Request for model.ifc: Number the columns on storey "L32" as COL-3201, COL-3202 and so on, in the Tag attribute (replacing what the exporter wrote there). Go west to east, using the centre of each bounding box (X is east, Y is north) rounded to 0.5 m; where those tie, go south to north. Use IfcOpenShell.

First a look at what the model holds.

```python
import ifcopenshell
import ifcopenshell.util.element
import ifcopenshell.util.placement

model = ifcopenshell.open("model.ifc")
print(model.schema)
storey = next(s for s in model.by_type("IfcBuildingStorey") if s.Name == "L32")
columns = [e for e in ifcopenshell.util.element.get_decomposition(storey) if e.is_a("IfcColumn")]
for e in sorted(columns, key=lambda e: e.id()):
    origin = ifcopenshell.util.placement.get_local_placement(e.ObjectPlacement)[:3, 3]
    print(e.id(), e.Tag, e.Name, origin.round(2) + 0.0, sep=" | ")
```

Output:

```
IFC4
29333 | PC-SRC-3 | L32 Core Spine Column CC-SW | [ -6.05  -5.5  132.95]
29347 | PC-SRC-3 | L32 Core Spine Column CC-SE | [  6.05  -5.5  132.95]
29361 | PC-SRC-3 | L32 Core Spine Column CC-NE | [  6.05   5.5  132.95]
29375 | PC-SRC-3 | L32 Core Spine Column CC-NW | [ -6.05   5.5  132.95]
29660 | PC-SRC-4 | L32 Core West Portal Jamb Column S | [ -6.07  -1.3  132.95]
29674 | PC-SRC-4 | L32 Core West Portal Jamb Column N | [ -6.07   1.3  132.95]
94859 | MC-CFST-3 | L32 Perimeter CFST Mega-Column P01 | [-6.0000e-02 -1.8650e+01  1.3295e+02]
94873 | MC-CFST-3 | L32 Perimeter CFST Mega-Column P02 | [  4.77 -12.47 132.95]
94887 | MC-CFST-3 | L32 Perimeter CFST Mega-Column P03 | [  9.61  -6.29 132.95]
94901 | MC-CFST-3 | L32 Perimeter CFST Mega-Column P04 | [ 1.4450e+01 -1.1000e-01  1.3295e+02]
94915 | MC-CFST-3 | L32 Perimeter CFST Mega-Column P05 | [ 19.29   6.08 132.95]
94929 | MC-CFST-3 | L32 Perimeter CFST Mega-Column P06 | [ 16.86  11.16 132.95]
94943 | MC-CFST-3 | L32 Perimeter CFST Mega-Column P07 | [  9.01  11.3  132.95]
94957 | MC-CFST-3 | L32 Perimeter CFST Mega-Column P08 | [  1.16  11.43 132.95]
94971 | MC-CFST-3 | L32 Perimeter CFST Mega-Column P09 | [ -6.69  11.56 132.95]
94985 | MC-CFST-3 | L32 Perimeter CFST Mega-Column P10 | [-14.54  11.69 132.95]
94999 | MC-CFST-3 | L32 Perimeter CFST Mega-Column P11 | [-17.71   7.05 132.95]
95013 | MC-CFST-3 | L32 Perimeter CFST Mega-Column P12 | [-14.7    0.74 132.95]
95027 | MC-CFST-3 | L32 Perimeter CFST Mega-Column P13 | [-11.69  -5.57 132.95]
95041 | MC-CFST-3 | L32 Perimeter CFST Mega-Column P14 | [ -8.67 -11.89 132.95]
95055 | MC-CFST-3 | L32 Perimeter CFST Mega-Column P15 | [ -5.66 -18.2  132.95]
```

```python
import ifcopenshell
import ifcopenshell.geom
import ifcopenshell.util.element
import ifcopenshell.util.shape

model = ifcopenshell.open("model.ifc")
settings = ifcopenshell.geom.settings()
settings.set("use-world-coords", True)


def centre(element):
    shape = ifcopenshell.geom.create_shape(settings, element)
    return ifcopenshell.util.shape.get_bbox_centroid(shape.geometry)


storey = next(s for s in model.by_type("IfcBuildingStorey") if s.Name == "L32")
columns = [e for e in ifcopenshell.util.element.get_decomposition(storey) if e.is_a("IfcColumn")]

# Insertion points can sit at a corner or the storey origin, so sort by the geometry (in metres).
centres = {e: centre(e) for e in columns}
columns.sort(key=lambda e: (round(centres[e][0] / 0.5), centres[e][1]))

for i, e in enumerate(columns, start=1):
    number = f"COL-32{i:02d}"
    e.Tag = number
    print(e.id(), number)

model.write("model_edited.ifc")
```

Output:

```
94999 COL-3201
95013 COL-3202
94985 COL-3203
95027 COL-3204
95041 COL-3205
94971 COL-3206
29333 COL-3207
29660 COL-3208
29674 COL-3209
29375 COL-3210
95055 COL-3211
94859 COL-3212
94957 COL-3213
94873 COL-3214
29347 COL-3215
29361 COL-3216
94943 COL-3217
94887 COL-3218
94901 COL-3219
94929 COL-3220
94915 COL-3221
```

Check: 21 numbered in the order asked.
